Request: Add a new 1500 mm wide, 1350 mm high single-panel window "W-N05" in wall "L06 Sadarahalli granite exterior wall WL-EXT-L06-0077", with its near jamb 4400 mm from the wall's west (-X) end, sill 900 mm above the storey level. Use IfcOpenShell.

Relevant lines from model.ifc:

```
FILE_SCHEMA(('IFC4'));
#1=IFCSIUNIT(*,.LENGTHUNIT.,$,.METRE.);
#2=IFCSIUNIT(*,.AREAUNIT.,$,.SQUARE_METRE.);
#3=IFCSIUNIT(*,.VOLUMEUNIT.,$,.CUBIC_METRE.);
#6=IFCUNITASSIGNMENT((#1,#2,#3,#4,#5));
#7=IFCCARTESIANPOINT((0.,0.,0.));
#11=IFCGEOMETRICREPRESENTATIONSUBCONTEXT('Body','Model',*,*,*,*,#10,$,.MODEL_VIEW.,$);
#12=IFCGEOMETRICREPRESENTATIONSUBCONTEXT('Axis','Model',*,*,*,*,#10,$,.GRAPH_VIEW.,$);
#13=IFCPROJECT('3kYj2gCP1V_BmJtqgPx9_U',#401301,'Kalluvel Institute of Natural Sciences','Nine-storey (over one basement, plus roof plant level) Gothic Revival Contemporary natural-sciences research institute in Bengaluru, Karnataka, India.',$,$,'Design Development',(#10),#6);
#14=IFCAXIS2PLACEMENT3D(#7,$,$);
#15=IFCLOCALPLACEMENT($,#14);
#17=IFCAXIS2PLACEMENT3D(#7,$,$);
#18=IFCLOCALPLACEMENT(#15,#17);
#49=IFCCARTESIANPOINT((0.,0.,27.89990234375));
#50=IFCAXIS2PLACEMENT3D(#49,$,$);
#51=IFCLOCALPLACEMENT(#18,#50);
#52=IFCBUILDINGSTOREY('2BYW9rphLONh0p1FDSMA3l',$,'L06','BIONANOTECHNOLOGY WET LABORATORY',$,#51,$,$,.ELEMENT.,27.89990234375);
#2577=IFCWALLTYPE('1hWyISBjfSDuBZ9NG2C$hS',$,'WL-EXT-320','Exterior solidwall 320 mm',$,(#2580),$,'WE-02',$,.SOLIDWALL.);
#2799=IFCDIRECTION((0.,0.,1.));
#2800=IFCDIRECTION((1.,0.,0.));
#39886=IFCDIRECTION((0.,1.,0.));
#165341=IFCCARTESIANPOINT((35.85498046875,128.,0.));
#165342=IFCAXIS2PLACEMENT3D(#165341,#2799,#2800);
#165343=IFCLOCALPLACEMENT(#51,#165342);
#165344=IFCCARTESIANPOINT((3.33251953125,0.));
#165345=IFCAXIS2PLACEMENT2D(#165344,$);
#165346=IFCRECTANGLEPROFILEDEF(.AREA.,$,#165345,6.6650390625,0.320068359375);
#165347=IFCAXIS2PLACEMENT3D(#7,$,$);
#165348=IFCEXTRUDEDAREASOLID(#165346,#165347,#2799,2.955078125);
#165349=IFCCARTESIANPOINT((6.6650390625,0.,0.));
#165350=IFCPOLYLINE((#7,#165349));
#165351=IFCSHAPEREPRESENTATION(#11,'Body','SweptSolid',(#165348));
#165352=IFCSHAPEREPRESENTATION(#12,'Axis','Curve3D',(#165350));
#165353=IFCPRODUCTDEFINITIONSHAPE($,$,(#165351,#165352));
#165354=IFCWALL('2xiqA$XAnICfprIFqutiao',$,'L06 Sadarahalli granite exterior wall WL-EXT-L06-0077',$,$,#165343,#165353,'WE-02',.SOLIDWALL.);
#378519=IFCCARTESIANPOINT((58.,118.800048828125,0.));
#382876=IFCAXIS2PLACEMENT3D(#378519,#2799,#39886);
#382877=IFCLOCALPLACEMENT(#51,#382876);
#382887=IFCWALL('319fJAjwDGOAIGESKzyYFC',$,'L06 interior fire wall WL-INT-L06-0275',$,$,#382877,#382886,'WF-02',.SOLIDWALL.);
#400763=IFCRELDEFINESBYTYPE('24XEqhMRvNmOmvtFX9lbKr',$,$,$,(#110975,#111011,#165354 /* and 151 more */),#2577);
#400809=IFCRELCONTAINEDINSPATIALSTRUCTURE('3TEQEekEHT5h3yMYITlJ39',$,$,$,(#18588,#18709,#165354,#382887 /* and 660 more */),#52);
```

```python
import numpy as np
import ifcopenshell
import ifcopenshell.api.feature
import ifcopenshell.api.geometry
import ifcopenshell.api.root
import ifcopenshell.api.spatial
import ifcopenshell.geom
import ifcopenshell.util.element
import ifcopenshell.util.placement
import ifcopenshell.util.representation
import ifcopenshell.util.shape
import ifcopenshell.util.unit

model = ifcopenshell.open("model.ifc")
unit_scale = ifcopenshell.util.unit.calculate_unit_scale(model)
settings = ifcopenshell.geom.settings()


def volume(element):
    """Net volume in cubic metres, openings subtracted."""
    shape = ifcopenshell.geom.create_shape(settings, element)
    return ifcopenshell.util.shape.get_volume(shape.geometry)


wall = model.by_guid("2xiqA$XAnICfprIFqutiao")
storey = ifcopenshell.util.element.get_container(wall, ifc_class="IfcBuildingStorey")
context = ifcopenshell.util.representation.get_context(model, "Model", "Body", "MODEL_VIEW")
before = volume(wall)

width, height, from_end, sill = 1.5, 1.35, 4.4, 0.9  # metres

# The wall runs along its own X axis, and the end named is its -X end.
wall_shape = ifcopenshell.geom.create_shape(settings, wall)
x, y, z = ifcopenshell.util.shape.get_vertices(wall_shape.geometry).T
start = x.min() + from_end
face, thickness = float(y.min()), float(y.max() - y.min())
wall_matrix = ifcopenshell.util.placement.get_local_placement(wall.ObjectPlacement)
level = ifcopenshell.util.placement.get_local_placement(storey.ObjectPlacement)[2, 3]


def in_wall(x, y):
    """Placement at x, y metres in the wall's axes, at sill height."""
    matrix = wall_matrix.copy()
    matrix[:, 3] = wall_matrix @ np.array([x / unit_scale, y / unit_scale, 0.0, 1.0])
    matrix[2, 3] = level + sill / unit_scale
    return matrix


# Opening: a box that overshoots both wall faces by 50 mm.
opening = ifcopenshell.api.root.create_entity(model, ifc_class="IfcOpeningElement", predefined_type="OPENING")
box = ifcopenshell.api.geometry.add_wall_representation(
    model, context=context, length=width, height=height, thickness=thickness + 0.1
)
ifcopenshell.api.geometry.assign_representation(model, product=opening, representation=box)
ifcopenshell.api.geometry.edit_object_placement(model, product=opening, matrix=in_wall(start, face - 0.05), is_si=False)
ifcopenshell.api.feature.add_feature(model, feature=opening, element=wall)

window = ifcopenshell.api.root.create_entity(model, ifc_class="IfcWindow", name="W-N05", predefined_type="WINDOW")
window.OverallWidth, window.OverallHeight = width / unit_scale, height / unit_scale
window.PartitioningType = "SINGLE_PANEL"
body = ifcopenshell.api.geometry.add_window_representation(
    model,
    context=context,
    overall_width=window.OverallWidth,
    overall_height=window.OverallHeight,
    partition_type="SINGLE_PANEL",
)
ifcopenshell.api.geometry.assign_representation(model, product=window, representation=body)
ifcopenshell.api.spatial.assign_container(model, products=[window], relating_structure=storey)
ifcopenshell.api.feature.add_filling(model, opening=opening, element=window)

# Centre the window in the wall's thickness.
ifcopenshell.api.geometry.edit_object_placement(model, product=window, matrix=in_wall(start, face), is_si=False)
window_shape = ifcopenshell.geom.create_shape(settings, window)
depth = ifcopenshell.util.shape.get_vertices(window_shape.geometry)[:, 1]
offset = face + thickness / 2 - (depth.min() + depth.max()) / 2
ifcopenshell.api.geometry.edit_object_placement(model, product=window, matrix=in_wall(start, offset), is_si=False)

after = volume(wall)

print(f"wall volume {before:.3f} -> {after:.3f} m3")

model.write("model_edited.ifc")
```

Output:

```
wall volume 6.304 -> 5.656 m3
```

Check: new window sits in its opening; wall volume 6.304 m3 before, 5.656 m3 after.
